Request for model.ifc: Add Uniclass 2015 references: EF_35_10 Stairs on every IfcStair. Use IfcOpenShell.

First a look at what the model holds.

```python
import ifcopenshell

model = ifcopenshell.open("model.ifc")
print(model.schema)
print("classifications:", [c.Name for c in model.by_type("IfcClassification")])
for ifc_class in ("IfcDoor", "IfcRoof", "IfcStair", "IfcWall", "IfcWindow"):
    print(ifc_class, len(model.by_type(ifc_class)))
```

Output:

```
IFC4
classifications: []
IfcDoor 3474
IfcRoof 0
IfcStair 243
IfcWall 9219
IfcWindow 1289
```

```python
import ifcopenshell
import ifcopenshell.api.classification

model = ifcopenshell.open("model.ifc")

system = ifcopenshell.api.classification.add_classification(model, classification="Uniclass 2015")

codes = {
    "IfcStair": ("EF_35_10", "Stairs"),
}
for ifc_class, (code, name) in codes.items():
    products = model.by_type(ifc_class)
    ifcopenshell.api.classification.add_reference(
        model, products=products, classification=system, identification=code, name=name
    )
    print(code, len(products))

model.write("model-out.ifc")
```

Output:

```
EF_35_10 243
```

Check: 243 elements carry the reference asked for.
